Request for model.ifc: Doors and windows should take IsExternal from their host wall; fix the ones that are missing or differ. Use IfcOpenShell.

First a look at what the model holds.

```python
import ifcopenshell
import ifcopenshell.util.element

model = ifcopenshell.open("model.ifc")
print(model.schema)
seen = {}
for e in model.by_type("IfcDoor") + model.by_type("IfcWindow"):
    if not e.FillsVoids:
        continue
    host = e.FillsVoids[0].RelatingOpeningElement.VoidsElements[0].RelatingBuildingElement
    own = ifcopenshell.util.element.get_pset(e, f"Pset_{e.is_a()[3:].removesuffix('StandardCase')}Common", "IsExternal")
    wall = ifcopenshell.util.element.get_pset(host, "Pset_WallCommon", "IsExternal")
    seen[e.is_a(), own, wall] = seen.get((e.is_a(), own, wall), 0) + 1
for (cls, own, wall), count in sorted(seen.items(), key=str):
    print(count, cls, "IsExternal:", own, "| host wall:", wall)
```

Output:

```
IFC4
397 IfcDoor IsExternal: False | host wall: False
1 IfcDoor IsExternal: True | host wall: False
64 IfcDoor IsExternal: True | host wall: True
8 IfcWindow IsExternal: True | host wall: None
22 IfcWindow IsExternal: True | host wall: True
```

```python
import ifcopenshell
import ifcopenshell.api.pset
import ifcopenshell.util.element

model = ifcopenshell.open("model.ifc")

count = 0
for ifc_class, pset_name in (("IfcDoor", "Pset_DoorCommon"), ("IfcWindow", "Pset_WindowCommon")):
    for e in model.by_type(ifc_class):
        if not e.FillsVoids:
            continue
        host = e.FillsVoids[0].RelatingOpeningElement.VoidsElements[0].RelatingBuildingElement
        external = ifcopenshell.util.element.get_pset(host, "Pset_WallCommon", "IsExternal")
        if external is None or ifcopenshell.util.element.get_pset(e, pset_name, "IsExternal") == external:
            continue
        pset = ifcopenshell.api.pset.add_pset(model, product=e, name=pset_name)
        ifcopenshell.api.pset.edit_pset(model, pset=pset, properties={"IsExternal": external})
        count += 1

print(count, "updated")

model.write("model_edited.ifc")
```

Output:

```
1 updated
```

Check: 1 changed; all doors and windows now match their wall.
